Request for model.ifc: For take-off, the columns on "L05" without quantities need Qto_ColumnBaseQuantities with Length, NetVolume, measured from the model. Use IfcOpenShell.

First a look at what the model holds.

```python
import ifcopenshell
import ifcopenshell.util.element
import ifcopenshell.util.unit

model = ifcopenshell.open("model.ifc")
print(model.schema)
for unit_type in ("LENGTHUNIT", "AREAUNIT", "VOLUMEUNIT"):
    print(unit_type, ifcopenshell.util.unit.calculate_unit_scale(model, unit_type))
storey = next(s for s in model.by_type("IfcBuildingStorey") if s.Name == "L05")
columns = [e for e in ifcopenshell.util.element.get_decomposition(storey) if e.is_a("IfcColumn")]
for e in sorted(columns, key=lambda e: e.id()):
    print(e.id(), e.is_a(), e.Name, list(ifcopenshell.util.element.get_psets(e, qtos_only=True)), sep=" | ")
```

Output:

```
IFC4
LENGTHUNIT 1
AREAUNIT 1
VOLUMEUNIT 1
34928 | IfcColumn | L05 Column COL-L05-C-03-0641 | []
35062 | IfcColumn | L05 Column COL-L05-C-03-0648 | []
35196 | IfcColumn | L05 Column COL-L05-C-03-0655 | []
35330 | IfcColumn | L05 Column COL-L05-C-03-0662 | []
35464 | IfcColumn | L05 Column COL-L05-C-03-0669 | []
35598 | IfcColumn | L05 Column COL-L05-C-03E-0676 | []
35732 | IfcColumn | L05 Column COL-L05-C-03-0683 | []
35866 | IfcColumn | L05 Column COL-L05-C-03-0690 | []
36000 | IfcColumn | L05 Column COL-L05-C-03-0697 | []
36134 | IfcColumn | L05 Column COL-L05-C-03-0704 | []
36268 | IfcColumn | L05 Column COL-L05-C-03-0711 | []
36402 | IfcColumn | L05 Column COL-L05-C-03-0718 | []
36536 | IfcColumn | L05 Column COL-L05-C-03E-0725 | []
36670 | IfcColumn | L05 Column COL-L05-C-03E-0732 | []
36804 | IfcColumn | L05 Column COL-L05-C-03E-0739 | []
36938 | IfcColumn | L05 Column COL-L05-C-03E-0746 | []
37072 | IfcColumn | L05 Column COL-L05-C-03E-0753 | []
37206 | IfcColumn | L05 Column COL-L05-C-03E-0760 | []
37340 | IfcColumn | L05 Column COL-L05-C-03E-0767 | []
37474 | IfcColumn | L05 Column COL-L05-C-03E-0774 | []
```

```python
import ifcopenshell
import ifcopenshell.api.pset
import ifcopenshell.geom
import ifcopenshell.util.element
import ifcopenshell.util.shape
import ifcopenshell.util.unit

model = ifcopenshell.open("model.ifc")
unit_scale = ifcopenshell.util.unit.calculate_unit_scale(model)
volume_scale = ifcopenshell.util.unit.calculate_unit_scale(model, "VOLUMEUNIT")
settings = ifcopenshell.geom.settings()

storey = next(s for s in model.by_type("IfcBuildingStorey") if s.Name == "L05")
columns = [e for e in ifcopenshell.util.element.get_decomposition(storey) if e.is_a("IfcColumn")]

for e in sorted(columns, key=lambda e: e.id()):
    if ifcopenshell.util.element.get_psets(e, qtos_only=True, should_inherit=False):
        continue
    # Geometry comes back in metres, in the element's own axes.
    shape = ifcopenshell.geom.create_shape(settings, e)
    values = {
        "Length": ifcopenshell.util.shape.get_z(shape.geometry) / unit_scale,
        "NetVolume": ifcopenshell.util.shape.get_volume(shape.geometry) / volume_scale,
    }
    qto = ifcopenshell.api.pset.add_qto(model, product=e, name="Qto_ColumnBaseQuantities")
    ifcopenshell.api.pset.edit_qto(model, qto=qto, properties=values)
    print(e.id(), {k: round(v, 3) for k, v in values.items()})

model.write("model_v2.ifc")
```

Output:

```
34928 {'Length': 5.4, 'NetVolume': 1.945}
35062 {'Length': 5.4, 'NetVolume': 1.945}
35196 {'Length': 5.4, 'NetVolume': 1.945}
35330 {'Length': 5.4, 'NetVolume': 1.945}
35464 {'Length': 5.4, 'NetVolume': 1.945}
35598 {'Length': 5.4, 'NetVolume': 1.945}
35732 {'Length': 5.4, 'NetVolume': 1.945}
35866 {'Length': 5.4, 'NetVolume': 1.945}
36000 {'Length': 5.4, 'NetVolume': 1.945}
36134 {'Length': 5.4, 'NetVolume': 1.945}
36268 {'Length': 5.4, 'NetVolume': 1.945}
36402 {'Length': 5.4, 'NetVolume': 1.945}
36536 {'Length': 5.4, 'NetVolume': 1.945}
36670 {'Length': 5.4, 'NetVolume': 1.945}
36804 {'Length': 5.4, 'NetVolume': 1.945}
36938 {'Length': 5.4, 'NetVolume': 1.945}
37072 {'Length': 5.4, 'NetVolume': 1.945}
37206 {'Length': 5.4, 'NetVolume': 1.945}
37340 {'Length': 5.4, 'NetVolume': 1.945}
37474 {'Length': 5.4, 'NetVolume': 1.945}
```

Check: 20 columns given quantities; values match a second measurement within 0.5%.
